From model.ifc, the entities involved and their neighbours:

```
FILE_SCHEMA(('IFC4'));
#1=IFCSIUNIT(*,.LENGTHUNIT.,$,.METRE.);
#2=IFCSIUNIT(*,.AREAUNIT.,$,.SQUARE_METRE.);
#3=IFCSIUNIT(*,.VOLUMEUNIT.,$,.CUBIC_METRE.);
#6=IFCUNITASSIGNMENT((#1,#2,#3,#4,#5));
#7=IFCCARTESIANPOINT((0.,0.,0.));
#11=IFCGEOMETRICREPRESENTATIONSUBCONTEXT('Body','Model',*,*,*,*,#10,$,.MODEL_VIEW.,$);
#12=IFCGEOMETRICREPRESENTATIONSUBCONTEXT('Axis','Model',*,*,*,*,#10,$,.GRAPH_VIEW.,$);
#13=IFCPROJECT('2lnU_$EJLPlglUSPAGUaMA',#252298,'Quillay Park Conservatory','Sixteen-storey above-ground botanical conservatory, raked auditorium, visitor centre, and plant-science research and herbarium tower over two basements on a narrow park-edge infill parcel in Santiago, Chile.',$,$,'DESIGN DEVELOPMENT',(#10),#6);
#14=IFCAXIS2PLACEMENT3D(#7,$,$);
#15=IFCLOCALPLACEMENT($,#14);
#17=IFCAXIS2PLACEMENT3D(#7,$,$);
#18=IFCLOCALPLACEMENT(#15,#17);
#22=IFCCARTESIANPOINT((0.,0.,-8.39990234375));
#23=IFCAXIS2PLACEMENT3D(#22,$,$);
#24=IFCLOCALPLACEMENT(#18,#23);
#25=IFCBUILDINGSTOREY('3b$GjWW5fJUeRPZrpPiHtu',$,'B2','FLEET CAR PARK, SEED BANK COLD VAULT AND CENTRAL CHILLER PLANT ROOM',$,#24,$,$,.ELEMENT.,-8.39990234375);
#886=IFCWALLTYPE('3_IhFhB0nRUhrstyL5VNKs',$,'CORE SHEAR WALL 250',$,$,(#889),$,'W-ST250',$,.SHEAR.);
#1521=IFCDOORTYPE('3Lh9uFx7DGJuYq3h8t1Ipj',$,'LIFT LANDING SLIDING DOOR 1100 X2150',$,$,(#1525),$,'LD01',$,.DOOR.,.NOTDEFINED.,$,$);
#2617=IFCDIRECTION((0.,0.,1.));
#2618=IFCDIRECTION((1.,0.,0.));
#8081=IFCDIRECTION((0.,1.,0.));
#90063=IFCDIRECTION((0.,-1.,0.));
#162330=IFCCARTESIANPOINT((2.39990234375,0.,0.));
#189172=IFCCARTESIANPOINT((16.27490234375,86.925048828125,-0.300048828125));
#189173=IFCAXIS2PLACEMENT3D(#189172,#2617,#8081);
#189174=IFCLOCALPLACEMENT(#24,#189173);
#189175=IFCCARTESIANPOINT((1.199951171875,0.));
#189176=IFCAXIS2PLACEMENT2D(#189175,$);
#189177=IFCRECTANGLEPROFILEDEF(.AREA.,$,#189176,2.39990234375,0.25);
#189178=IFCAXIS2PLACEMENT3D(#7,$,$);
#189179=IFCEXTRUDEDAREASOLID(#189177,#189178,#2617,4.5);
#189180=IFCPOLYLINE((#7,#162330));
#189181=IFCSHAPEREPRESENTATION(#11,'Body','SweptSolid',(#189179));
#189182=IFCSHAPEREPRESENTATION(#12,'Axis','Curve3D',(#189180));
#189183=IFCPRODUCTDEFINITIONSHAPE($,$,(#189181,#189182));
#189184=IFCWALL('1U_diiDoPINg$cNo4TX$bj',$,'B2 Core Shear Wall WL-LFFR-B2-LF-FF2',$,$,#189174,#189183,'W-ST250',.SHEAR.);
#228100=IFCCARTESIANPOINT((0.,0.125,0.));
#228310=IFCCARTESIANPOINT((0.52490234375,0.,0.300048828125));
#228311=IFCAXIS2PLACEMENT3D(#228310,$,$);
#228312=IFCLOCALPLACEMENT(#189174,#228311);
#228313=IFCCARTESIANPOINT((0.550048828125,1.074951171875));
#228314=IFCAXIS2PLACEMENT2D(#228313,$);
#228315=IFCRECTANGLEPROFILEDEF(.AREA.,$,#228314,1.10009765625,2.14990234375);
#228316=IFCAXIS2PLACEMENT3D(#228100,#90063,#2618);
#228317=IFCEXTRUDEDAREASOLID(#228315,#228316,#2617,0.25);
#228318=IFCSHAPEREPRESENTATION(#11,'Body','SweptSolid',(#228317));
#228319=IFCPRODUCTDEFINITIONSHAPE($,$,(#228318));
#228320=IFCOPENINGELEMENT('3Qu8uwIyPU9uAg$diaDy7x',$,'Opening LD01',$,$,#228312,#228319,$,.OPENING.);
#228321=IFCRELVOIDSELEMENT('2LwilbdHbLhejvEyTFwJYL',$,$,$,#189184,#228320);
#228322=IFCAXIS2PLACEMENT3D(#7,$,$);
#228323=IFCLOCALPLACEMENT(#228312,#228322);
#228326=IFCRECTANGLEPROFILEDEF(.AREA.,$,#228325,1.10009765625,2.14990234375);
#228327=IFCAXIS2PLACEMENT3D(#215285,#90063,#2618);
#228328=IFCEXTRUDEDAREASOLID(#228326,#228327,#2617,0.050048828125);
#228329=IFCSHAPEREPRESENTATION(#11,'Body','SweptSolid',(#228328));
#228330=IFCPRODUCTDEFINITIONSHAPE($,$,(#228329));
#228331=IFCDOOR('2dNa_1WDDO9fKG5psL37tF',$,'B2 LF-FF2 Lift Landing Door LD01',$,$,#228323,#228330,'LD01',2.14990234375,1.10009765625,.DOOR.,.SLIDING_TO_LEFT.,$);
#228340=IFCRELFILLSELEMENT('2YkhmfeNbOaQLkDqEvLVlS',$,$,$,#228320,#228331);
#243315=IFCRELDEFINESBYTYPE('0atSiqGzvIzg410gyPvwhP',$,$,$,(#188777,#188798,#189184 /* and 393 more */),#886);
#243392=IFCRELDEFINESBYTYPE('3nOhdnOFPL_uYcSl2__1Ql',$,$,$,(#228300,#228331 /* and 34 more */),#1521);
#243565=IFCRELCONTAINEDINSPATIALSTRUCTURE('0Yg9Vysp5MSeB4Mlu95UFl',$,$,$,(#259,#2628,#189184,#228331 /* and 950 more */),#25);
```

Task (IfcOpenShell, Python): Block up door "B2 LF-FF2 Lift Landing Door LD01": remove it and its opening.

```python
import ifcopenshell
import ifcopenshell.api.feature
import ifcopenshell.api.root
import ifcopenshell.geom
import ifcopenshell.util.shape

model = ifcopenshell.open("model.ifc")
settings = ifcopenshell.geom.settings()


def volume(element):
    """Net volume in cubic metres, openings subtracted."""
    shape = ifcopenshell.geom.create_shape(settings, element)
    return ifcopenshell.util.shape.get_volume(shape.geometry)


door = model.by_guid("2dNa_1WDDO9fKG5psL37tF")
opening = door.FillsVoids[0].RelatingOpeningElement
wall = opening.VoidsElements[0].RelatingBuildingElement
before = volume(wall)

ifcopenshell.api.root.remove_product(model, product=door)
ifcopenshell.api.feature.remove_feature(model, feature=opening)

after = volume(wall)

print(f"wall volume {before:.3f} -> {after:.3f} m3")

model.write("model_edited.ifc")
```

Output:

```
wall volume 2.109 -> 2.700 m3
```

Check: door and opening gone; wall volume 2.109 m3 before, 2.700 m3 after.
